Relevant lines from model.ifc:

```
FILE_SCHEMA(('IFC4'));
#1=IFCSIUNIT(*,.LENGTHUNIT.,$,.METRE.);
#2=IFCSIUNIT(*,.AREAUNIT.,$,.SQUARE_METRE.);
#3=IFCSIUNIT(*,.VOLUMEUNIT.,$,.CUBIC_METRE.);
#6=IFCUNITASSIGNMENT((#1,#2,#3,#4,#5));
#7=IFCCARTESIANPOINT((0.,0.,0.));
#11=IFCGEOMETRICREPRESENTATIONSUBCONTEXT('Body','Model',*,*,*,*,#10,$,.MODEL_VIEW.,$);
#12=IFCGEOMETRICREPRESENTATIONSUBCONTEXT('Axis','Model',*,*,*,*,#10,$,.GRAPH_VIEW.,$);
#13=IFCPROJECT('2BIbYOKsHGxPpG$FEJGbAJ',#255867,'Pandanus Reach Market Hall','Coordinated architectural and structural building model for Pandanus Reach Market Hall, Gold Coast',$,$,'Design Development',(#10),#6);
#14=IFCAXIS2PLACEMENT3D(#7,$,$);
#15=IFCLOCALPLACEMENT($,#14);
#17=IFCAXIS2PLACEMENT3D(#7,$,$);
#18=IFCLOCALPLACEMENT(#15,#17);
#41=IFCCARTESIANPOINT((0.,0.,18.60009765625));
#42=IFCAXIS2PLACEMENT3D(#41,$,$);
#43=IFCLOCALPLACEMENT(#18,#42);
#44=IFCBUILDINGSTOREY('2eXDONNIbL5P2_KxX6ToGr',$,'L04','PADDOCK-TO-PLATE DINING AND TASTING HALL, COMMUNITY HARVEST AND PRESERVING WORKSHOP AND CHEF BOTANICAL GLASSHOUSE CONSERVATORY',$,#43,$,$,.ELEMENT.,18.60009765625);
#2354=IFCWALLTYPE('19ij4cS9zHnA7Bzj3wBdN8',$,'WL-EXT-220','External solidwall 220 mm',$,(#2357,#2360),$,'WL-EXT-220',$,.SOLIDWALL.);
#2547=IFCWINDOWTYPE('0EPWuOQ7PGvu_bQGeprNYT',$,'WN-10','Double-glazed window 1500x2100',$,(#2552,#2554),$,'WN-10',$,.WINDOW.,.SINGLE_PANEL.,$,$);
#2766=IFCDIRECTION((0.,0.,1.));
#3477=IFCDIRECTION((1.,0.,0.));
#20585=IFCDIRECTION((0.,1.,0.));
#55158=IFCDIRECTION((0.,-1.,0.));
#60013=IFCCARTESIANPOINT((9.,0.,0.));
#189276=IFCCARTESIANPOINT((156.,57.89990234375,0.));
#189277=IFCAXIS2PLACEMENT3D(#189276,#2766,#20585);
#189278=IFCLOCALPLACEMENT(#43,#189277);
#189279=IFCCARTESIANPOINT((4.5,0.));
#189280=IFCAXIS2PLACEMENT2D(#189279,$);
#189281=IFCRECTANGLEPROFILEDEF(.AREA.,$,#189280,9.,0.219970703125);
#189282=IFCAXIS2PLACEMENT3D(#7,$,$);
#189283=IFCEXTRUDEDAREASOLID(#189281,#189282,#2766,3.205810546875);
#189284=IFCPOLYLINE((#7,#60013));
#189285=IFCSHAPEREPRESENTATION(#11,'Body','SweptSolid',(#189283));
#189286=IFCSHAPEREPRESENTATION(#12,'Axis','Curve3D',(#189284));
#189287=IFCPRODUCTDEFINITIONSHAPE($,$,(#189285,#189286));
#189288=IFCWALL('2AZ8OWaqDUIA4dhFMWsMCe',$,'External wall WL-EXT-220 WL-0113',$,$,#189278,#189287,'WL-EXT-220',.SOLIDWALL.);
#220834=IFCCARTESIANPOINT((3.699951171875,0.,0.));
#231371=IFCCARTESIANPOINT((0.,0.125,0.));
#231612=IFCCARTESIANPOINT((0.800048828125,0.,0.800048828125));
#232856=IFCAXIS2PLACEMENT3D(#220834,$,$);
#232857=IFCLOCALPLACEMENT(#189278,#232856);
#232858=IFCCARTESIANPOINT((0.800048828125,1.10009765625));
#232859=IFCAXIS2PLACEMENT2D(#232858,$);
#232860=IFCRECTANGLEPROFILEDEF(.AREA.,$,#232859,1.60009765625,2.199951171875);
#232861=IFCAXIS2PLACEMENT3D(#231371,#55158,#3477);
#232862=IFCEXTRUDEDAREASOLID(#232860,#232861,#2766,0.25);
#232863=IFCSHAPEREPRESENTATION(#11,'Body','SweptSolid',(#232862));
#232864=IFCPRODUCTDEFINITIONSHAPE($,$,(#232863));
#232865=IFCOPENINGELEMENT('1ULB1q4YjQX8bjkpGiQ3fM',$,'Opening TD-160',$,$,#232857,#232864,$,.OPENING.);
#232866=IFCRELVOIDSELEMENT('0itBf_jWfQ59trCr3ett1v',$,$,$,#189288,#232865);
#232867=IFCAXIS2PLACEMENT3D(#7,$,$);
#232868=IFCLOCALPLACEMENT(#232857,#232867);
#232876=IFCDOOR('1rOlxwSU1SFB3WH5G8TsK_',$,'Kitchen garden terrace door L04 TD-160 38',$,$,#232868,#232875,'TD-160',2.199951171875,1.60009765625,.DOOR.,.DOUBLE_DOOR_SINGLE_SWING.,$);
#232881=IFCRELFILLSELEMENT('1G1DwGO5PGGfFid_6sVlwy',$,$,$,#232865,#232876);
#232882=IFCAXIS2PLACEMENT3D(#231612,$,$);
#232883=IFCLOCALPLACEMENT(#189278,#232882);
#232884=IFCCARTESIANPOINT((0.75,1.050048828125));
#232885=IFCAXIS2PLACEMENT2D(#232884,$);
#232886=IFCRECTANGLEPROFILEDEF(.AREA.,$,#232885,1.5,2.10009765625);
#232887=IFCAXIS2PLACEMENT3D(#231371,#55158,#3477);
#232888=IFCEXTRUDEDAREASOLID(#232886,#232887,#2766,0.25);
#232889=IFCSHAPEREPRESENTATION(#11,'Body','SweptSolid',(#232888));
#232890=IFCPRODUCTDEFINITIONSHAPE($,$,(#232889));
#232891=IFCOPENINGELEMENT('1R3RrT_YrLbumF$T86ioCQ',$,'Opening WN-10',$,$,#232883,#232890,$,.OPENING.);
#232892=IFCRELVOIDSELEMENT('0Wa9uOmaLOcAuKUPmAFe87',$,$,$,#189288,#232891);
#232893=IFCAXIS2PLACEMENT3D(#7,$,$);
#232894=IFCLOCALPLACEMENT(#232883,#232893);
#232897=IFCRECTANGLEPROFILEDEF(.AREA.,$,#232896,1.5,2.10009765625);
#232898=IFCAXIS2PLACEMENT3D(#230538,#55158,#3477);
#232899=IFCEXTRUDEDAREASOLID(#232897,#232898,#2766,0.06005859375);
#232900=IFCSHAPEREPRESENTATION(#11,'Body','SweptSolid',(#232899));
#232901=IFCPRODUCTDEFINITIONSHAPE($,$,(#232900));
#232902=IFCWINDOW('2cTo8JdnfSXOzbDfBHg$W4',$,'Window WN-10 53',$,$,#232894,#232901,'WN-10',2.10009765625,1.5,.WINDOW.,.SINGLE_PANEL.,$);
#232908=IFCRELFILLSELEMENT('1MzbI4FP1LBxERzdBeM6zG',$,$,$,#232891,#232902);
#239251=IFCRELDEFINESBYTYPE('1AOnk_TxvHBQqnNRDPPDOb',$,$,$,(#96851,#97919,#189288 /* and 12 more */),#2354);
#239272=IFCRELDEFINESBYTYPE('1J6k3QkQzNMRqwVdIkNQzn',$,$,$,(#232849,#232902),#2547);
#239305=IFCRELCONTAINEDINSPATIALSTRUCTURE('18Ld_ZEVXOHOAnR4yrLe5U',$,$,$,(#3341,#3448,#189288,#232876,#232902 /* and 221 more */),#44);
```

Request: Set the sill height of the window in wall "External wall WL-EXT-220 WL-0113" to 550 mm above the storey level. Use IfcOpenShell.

```python
import numpy as np
import ifcopenshell
import ifcopenshell.api.geometry
import ifcopenshell.geom
import ifcopenshell.util.element
import ifcopenshell.util.placement
import ifcopenshell.util.shape
import ifcopenshell.util.unit

model = ifcopenshell.open("model.ifc")
unit_scale = ifcopenshell.util.unit.calculate_unit_scale(model)

window = model.by_guid("2cTo8JdnfSXOzbDfBHg$W4")
opening = window.FillsVoids[0].RelatingOpeningElement
storey = ifcopenshell.util.element.get_container(window, ifc_class="IfcBuildingStorey")
level = ifcopenshell.util.placement.get_local_placement(storey.ObjectPlacement)[2, 3]

# The opening's origin need not be at the sill, so measure its lowest point.
shape = ifcopenshell.geom.create_shape(ifcopenshell.geom.settings(), opening)
bottom = ifcopenshell.util.shape.get_shape_bottom_elevation(shape, shape.geometry) / unit_scale
dz = level + 0.55 / unit_scale - bottom

shift = np.array([0.0, 0.0, dz])
# The window is placed relative to its opening, so it follows when the opening moves.
matrix = ifcopenshell.util.placement.get_local_placement(opening.ObjectPlacement)
matrix[:3, 3] += shift
ifcopenshell.api.geometry.edit_object_placement(
    model, product=opening, matrix=matrix, is_si=False, should_transform_children=True
)

print(f"moved by {dz * unit_scale:+.3f} m")

model.write("model-out.ifc")
```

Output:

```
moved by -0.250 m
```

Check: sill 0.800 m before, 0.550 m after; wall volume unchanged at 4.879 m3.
